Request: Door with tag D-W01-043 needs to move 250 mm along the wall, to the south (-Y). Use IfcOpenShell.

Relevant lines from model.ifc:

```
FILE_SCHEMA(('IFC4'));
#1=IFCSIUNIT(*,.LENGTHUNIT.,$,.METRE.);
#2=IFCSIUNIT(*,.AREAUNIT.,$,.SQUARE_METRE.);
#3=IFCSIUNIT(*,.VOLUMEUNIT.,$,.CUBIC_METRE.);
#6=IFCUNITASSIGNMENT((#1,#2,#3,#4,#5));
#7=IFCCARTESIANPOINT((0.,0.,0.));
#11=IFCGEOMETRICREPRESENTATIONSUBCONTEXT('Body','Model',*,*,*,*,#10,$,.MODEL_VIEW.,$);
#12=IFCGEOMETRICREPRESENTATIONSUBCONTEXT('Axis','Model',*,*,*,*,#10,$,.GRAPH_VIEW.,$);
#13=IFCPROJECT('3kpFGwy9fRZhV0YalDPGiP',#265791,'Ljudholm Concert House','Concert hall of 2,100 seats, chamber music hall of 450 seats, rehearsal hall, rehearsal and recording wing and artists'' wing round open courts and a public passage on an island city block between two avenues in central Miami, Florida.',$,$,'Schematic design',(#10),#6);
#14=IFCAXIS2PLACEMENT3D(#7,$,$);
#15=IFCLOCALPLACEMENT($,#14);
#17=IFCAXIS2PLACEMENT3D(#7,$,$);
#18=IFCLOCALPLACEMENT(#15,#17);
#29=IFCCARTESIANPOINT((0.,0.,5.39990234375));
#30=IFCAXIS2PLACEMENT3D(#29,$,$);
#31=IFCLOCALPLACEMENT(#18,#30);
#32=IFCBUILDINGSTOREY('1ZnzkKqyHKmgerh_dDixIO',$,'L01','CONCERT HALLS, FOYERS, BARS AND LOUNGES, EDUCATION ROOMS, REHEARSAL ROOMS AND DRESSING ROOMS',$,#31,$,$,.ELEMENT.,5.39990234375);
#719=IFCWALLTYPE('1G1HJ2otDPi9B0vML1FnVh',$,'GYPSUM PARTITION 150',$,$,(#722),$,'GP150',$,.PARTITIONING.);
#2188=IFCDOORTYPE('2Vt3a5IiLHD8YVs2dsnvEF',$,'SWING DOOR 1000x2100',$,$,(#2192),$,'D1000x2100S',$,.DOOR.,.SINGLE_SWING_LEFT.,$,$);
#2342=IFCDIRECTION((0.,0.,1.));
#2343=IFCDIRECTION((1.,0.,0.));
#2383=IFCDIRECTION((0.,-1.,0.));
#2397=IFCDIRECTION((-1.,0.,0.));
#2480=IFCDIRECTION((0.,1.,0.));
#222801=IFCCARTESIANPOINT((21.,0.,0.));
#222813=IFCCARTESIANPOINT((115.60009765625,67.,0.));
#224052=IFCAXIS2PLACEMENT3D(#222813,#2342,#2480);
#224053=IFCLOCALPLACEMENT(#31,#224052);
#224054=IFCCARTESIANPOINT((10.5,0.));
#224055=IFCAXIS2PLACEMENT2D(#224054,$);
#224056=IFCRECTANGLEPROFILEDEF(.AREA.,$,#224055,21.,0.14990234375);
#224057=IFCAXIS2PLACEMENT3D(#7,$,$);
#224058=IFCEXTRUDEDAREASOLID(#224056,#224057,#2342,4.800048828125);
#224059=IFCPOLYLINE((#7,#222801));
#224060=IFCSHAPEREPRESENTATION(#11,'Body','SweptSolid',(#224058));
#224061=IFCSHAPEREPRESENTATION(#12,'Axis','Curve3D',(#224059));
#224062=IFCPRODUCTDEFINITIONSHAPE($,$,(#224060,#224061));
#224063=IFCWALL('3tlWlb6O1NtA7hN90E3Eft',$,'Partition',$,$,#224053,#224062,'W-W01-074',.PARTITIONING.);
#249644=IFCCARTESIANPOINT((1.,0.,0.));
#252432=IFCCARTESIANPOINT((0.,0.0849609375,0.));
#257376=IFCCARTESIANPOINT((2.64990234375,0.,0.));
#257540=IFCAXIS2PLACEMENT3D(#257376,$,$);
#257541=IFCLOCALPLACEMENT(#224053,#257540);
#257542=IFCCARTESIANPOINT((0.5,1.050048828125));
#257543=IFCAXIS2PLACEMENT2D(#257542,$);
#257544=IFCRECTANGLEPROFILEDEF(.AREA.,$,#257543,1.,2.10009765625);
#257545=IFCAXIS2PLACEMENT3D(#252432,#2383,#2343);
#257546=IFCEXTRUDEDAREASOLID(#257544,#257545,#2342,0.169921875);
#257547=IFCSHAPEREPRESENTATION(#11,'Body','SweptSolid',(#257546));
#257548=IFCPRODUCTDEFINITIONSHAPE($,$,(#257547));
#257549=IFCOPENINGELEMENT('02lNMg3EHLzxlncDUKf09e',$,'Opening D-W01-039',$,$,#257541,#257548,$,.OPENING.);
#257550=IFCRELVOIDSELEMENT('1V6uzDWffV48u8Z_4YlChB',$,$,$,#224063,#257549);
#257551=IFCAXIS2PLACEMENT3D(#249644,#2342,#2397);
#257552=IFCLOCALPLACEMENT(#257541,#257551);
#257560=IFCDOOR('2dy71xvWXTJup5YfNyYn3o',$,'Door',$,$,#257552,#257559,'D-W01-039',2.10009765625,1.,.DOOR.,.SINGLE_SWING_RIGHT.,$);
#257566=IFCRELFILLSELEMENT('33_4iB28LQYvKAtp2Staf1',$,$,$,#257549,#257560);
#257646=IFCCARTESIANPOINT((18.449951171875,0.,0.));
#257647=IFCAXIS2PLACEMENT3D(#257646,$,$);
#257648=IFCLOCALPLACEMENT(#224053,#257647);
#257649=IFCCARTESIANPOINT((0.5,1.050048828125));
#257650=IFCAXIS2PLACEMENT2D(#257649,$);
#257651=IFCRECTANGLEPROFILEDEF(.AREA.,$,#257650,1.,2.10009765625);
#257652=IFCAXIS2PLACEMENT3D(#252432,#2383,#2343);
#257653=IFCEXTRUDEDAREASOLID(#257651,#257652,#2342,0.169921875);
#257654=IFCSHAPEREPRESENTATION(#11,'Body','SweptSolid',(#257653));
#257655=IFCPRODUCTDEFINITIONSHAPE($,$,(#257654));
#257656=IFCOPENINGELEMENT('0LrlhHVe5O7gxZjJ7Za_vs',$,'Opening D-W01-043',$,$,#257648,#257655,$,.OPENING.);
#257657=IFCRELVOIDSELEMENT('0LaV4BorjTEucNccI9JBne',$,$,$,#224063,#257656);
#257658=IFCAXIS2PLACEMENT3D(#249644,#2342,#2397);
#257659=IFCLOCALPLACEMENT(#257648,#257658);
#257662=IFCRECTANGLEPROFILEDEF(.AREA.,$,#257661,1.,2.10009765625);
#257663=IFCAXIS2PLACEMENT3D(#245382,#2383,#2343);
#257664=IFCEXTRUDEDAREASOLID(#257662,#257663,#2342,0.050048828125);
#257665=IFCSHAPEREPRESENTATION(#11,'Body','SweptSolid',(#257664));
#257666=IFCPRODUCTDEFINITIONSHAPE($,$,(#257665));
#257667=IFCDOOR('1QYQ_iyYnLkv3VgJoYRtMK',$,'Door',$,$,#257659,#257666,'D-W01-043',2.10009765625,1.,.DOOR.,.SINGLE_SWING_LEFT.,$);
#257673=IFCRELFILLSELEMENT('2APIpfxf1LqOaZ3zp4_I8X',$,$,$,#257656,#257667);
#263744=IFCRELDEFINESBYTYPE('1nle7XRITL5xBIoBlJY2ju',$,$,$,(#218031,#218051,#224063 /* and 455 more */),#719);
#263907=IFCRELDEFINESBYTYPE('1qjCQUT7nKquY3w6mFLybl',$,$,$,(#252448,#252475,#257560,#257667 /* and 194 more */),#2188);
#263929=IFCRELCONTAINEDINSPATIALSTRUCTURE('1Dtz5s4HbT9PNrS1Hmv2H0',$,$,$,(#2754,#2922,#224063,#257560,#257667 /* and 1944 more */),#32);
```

```python
import ifcopenshell
import ifcopenshell.api.geometry
import ifcopenshell.util.placement
import ifcopenshell.util.unit

model = ifcopenshell.open("model.ifc")
unit_scale = ifcopenshell.util.unit.calculate_unit_scale(model)

door = model.by_id(257667)
opening = door.FillsVoids[0].RelatingOpeningElement
wall = opening.VoidsElements[0].RelatingBuildingElement

wall_matrix = ifcopenshell.util.placement.get_local_placement(wall.ObjectPlacement)
shift = wall_matrix[:3, 0] * -0.25 / unit_scale
before = ifcopenshell.util.placement.get_local_placement(door.ObjectPlacement)[:3, 3].copy()

# The door is placed relative to its opening, so it follows when the opening moves.
matrix = ifcopenshell.util.placement.get_local_placement(opening.ObjectPlacement)
matrix[:3, 3] += shift
ifcopenshell.api.geometry.edit_object_placement(
    model, product=opening, matrix=matrix, is_si=False, should_transform_children=True
)

after = ifcopenshell.util.placement.get_local_placement(door.ObjectPlacement)[:3, 3]
print("door moved by", (after - before).round(3) + 0.0)

model.write("model_edited.ifc")
```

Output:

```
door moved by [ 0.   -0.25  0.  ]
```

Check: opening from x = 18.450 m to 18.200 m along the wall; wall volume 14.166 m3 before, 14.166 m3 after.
